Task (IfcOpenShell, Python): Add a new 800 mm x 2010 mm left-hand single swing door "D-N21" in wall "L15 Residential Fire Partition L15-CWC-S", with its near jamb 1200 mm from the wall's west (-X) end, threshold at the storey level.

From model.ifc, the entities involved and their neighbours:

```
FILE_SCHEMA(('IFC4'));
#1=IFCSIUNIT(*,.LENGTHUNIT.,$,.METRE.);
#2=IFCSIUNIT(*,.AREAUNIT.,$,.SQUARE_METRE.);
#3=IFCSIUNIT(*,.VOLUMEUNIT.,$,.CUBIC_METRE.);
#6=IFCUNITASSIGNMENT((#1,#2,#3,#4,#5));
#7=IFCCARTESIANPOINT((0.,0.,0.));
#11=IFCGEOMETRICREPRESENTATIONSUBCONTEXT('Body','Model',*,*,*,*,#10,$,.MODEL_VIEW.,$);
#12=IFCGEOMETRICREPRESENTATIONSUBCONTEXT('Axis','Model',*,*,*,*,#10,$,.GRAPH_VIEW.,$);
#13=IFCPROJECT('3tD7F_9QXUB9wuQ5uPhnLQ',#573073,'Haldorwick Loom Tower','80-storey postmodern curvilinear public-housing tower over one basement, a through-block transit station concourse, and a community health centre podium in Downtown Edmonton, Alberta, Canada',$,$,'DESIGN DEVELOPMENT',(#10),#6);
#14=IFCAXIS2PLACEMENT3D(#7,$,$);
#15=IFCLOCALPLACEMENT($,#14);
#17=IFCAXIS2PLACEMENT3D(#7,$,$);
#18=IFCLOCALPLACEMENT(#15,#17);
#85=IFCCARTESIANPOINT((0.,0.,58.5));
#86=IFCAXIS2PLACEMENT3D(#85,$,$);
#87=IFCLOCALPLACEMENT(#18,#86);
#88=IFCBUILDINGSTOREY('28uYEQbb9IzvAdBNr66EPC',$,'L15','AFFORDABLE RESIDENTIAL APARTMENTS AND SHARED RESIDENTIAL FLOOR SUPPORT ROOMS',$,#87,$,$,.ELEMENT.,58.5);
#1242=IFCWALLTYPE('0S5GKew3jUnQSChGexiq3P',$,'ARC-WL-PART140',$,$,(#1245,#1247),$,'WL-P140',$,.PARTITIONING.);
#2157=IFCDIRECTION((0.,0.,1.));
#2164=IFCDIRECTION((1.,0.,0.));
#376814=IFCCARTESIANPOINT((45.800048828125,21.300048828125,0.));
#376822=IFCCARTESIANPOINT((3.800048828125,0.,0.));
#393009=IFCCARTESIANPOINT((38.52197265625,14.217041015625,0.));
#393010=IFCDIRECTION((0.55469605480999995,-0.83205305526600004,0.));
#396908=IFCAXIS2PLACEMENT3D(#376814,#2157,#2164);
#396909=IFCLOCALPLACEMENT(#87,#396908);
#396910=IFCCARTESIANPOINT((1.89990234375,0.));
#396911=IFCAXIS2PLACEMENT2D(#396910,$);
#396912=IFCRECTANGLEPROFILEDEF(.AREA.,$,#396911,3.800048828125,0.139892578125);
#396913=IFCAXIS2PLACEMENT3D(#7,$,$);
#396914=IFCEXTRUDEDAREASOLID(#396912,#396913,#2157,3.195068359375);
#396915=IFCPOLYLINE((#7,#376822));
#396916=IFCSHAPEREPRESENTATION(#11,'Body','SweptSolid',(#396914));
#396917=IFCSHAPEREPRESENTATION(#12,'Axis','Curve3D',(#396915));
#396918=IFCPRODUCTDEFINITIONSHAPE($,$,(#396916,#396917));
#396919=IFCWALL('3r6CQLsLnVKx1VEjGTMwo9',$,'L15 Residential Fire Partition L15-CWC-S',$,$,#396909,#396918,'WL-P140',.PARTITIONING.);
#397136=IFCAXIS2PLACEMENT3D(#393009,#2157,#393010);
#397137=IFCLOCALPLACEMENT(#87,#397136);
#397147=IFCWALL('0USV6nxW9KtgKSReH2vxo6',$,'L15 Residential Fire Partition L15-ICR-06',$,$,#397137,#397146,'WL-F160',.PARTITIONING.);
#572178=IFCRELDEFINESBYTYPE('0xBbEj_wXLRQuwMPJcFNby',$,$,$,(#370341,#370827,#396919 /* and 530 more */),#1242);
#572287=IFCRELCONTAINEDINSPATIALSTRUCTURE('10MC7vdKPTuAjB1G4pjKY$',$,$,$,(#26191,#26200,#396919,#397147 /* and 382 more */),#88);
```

```python
import numpy as np
import ifcopenshell
import ifcopenshell.api.feature
import ifcopenshell.api.geometry
import ifcopenshell.api.root
import ifcopenshell.api.spatial
import ifcopenshell.geom
import ifcopenshell.util.element
import ifcopenshell.util.placement
import ifcopenshell.util.representation
import ifcopenshell.util.shape
import ifcopenshell.util.unit

model = ifcopenshell.open("model.ifc")
unit_scale = ifcopenshell.util.unit.calculate_unit_scale(model)
settings = ifcopenshell.geom.settings()


def volume(element):
    """Net volume in cubic metres, openings subtracted."""
    shape = ifcopenshell.geom.create_shape(settings, element)
    return ifcopenshell.util.shape.get_volume(shape.geometry)


wall = model.by_id(396919)
storey = ifcopenshell.util.element.get_container(wall, ifc_class="IfcBuildingStorey")
context = ifcopenshell.util.representation.get_context(model, "Model", "Body", "MODEL_VIEW")
before = volume(wall)

width, height, from_end, sill = 0.8, 2.01, 1.2, 0.0  # metres

# The wall runs along its own X axis, and the end named is its -X end.
wall_shape = ifcopenshell.geom.create_shape(settings, wall)
x, y, z = ifcopenshell.util.shape.get_vertices(wall_shape.geometry).T
start = x.min() + from_end
face, thickness = float(y.min()), float(y.max() - y.min())
wall_matrix = ifcopenshell.util.placement.get_local_placement(wall.ObjectPlacement)
level = ifcopenshell.util.placement.get_local_placement(storey.ObjectPlacement)[2, 3]


def in_wall(x, y):
    """Placement at x, y metres in the wall's axes, at sill height."""
    matrix = wall_matrix.copy()
    matrix[:, 3] = wall_matrix @ np.array([x / unit_scale, y / unit_scale, 0.0, 1.0])
    matrix[2, 3] = level + sill / unit_scale
    return matrix


# Opening: a box that overshoots both wall faces by 50 mm.
opening = ifcopenshell.api.root.create_entity(model, ifc_class="IfcOpeningElement", predefined_type="OPENING")
box = ifcopenshell.api.geometry.add_wall_representation(
    model, context=context, length=width, height=height, thickness=thickness + 0.1
)
ifcopenshell.api.geometry.assign_representation(model, product=opening, representation=box)
ifcopenshell.api.geometry.edit_object_placement(model, product=opening, matrix=in_wall(start, face - 0.05), is_si=False)
ifcopenshell.api.feature.add_feature(model, feature=opening, element=wall)

door = ifcopenshell.api.root.create_entity(model, ifc_class="IfcDoor", name="D-N21", predefined_type="DOOR")
door.OverallWidth, door.OverallHeight = width / unit_scale, height / unit_scale
door.OperationType = "SINGLE_SWING_LEFT"
body = ifcopenshell.api.geometry.add_door_representation(
    model,
    context=context,
    overall_width=door.OverallWidth,
    overall_height=door.OverallHeight,
    operation_type="SINGLE_SWING_LEFT",
    lining_properties={"LiningDepth": thickness / unit_scale, "ThresholdDepth": thickness / unit_scale},
)
ifcopenshell.api.geometry.assign_representation(model, product=door, representation=body)
ifcopenshell.api.spatial.assign_container(model, products=[door], relating_structure=storey)
ifcopenshell.api.feature.add_filling(model, opening=opening, element=door)

# The lining spans the wall, so the door starts at the wall face.
ifcopenshell.api.geometry.edit_object_placement(model, product=door, matrix=in_wall(start, face), is_si=False)

after = volume(wall)

print(f"wall volume {before:.3f} -> {after:.3f} m3")

model.write("model_edited.ifc")
```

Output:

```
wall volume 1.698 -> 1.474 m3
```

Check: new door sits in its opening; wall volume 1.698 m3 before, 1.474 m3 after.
